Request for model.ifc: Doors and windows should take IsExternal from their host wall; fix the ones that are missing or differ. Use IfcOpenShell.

First a look at what the model holds.

```python
import ifcopenshell
import ifcopenshell.util.element

model = ifcopenshell.open("model.ifc")
print(model.schema)
seen = {}
for e in model.by_type("IfcDoor") + model.by_type("IfcWindow"):
    if not e.FillsVoids:
        continue
    host = e.FillsVoids[0].RelatingOpeningElement.VoidsElements[0].RelatingBuildingElement
    own = ifcopenshell.util.element.get_pset(e, f"Pset_{e.is_a()[3:].removesuffix('StandardCase')}Common", "IsExternal")
    wall = ifcopenshell.util.element.get_pset(host, "Pset_WallCommon", "IsExternal")
    seen[e.is_a(), own, wall] = seen.get((e.is_a(), own, wall), 0) + 1
for (cls, own, wall), count in sorted(seen.items(), key=str):
    print(count, cls, "IsExternal:", own, "| host wall:", wall)
```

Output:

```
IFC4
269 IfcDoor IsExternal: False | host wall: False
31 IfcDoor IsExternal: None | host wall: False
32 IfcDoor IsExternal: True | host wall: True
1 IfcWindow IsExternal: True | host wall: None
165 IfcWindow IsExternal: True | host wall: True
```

```python
import ifcopenshell
import ifcopenshell.api.pset
import ifcopenshell.util.element

model = ifcopenshell.open("model.ifc")

count = 0
for ifc_class, pset_name in (("IfcDoor", "Pset_DoorCommon"), ("IfcWindow", "Pset_WindowCommon")):
    for e in model.by_type(ifc_class):
        if not e.FillsVoids:
            continue
        host = e.FillsVoids[0].RelatingOpeningElement.VoidsElements[0].RelatingBuildingElement
        external = ifcopenshell.util.element.get_pset(host, "Pset_WallCommon", "IsExternal")
        if external is None or ifcopenshell.util.element.get_pset(e, pset_name, "IsExternal") == external:
            continue
        pset = ifcopenshell.api.pset.add_pset(model, product=e, name=pset_name)
        ifcopenshell.api.pset.edit_pset(model, pset=pset, properties={"IsExternal": external})
        count += 1

print(count, "updated")

model.write("model_rev.ifc")
```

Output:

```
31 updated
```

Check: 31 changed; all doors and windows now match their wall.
